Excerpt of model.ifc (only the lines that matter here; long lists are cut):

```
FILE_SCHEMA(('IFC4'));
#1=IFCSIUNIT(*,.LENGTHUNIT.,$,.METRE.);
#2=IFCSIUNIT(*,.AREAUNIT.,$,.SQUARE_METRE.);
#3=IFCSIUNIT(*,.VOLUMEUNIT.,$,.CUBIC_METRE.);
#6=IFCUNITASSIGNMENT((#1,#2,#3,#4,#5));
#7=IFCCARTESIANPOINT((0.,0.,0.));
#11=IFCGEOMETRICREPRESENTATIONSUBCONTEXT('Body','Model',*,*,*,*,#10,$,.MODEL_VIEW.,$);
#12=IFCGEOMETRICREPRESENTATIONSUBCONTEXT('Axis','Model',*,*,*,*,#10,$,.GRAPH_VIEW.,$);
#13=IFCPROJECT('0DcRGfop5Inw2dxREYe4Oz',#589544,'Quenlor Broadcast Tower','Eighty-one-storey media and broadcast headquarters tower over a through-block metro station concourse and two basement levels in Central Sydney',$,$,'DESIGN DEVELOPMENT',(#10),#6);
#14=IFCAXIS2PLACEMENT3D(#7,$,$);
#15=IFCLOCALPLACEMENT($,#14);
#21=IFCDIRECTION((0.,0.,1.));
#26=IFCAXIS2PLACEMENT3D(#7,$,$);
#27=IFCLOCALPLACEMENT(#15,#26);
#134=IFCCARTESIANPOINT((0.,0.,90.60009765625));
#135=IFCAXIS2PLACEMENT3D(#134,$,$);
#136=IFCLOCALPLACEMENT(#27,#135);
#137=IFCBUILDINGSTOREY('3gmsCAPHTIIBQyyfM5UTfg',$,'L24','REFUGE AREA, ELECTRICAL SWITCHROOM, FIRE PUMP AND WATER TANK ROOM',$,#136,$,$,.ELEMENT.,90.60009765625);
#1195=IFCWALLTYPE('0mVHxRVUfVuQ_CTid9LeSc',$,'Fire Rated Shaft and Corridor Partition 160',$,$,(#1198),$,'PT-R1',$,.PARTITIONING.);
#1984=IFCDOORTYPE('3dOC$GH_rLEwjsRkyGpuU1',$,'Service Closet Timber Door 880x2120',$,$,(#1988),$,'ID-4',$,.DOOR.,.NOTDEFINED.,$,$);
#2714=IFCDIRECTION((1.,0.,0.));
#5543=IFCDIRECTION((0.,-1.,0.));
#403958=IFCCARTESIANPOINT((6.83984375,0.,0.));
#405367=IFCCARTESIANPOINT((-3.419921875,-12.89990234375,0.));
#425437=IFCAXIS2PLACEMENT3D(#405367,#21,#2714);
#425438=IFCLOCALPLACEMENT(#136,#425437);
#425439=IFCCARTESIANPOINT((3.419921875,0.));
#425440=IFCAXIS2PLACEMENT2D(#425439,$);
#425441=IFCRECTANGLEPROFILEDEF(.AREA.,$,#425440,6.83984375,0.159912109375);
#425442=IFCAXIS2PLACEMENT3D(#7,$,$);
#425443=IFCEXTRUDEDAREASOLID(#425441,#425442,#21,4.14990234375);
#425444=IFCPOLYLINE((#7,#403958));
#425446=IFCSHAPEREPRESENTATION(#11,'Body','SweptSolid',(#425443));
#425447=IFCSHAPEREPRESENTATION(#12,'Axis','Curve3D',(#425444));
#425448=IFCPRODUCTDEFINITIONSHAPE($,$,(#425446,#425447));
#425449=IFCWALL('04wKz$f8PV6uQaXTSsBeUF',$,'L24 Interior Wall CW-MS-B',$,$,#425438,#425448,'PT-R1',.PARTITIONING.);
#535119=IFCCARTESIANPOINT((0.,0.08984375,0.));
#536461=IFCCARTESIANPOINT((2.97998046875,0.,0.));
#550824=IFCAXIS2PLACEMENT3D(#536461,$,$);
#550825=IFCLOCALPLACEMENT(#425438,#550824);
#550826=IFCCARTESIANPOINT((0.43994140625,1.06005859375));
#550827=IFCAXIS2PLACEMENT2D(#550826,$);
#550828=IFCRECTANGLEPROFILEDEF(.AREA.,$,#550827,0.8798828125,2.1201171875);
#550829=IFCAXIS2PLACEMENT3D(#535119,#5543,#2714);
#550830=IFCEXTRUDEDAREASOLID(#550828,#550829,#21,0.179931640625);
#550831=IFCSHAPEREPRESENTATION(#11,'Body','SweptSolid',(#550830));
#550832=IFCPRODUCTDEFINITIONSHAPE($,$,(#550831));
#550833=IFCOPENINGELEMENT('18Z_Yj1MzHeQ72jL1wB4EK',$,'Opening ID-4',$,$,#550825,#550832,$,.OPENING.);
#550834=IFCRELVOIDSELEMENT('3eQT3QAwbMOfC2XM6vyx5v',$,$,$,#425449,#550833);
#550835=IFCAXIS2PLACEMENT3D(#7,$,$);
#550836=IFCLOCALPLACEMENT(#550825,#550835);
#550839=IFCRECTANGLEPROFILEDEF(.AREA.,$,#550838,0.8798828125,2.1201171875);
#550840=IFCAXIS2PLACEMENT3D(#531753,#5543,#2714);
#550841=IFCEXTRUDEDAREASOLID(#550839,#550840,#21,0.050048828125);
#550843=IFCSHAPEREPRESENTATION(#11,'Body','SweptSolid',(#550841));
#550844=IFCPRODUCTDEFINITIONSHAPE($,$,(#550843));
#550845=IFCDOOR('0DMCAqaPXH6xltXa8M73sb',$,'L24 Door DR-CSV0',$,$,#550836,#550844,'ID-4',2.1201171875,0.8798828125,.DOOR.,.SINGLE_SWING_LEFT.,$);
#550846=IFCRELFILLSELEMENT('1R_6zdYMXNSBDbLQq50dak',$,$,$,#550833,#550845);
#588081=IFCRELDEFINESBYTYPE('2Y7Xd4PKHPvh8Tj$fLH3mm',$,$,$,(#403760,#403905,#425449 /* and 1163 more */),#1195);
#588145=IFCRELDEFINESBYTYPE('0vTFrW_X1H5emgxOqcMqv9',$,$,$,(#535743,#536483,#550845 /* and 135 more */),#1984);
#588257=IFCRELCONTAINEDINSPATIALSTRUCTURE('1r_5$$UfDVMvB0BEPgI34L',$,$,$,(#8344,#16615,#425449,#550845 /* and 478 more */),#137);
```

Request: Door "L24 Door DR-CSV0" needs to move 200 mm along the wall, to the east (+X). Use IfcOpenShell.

```python
import ifcopenshell
import ifcopenshell.api.geometry
import ifcopenshell.util.placement

model = ifcopenshell.open("model.ifc")

door = model.by_guid("0DMCAqaPXH6xltXa8M73sb")
opening = door.FillsVoids[0].RelatingOpeningElement
wall = opening.VoidsElements[0].RelatingBuildingElement

wall_matrix = ifcopenshell.util.placement.get_local_placement(wall.ObjectPlacement)
shift = wall_matrix[:3, 0] * 0.2
before = ifcopenshell.util.placement.get_local_placement(door.ObjectPlacement)[:3, 3].copy()

# The door is placed relative to its opening, so it follows when the opening moves.
matrix = ifcopenshell.util.placement.get_local_placement(opening.ObjectPlacement)
matrix[:3, 3] += shift
ifcopenshell.api.geometry.edit_object_placement(
    model, product=opening, matrix=matrix, is_si=False, should_transform_children=True
)

after = ifcopenshell.util.placement.get_local_placement(door.ObjectPlacement)[:3, 3]
print("door moved by", (after - before).round(3) + 0.0)

model.write("model_edited.ifc")
```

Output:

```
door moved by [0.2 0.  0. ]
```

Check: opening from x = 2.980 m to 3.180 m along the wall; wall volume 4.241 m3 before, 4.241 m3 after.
